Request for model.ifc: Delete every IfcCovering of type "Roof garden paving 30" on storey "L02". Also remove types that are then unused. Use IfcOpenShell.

First a look at what the model holds.

```python
import ifcopenshell
import ifcopenshell.util.element

model = ifcopenshell.open("model.ifc")
print(model.schema)
storey = next(s for s in model.by_type("IfcBuildingStorey") if s.Name == "L02")
coverings = [e for e in ifcopenshell.util.element.get_decomposition(storey) if e.is_a("IfcCovering")]
seen = {}
for e in coverings:
    element_type = ifcopenshell.util.element.get_type(e)
    name = element_type.Name if element_type not in (None, e) else None
    seen[name] = seen.get(name, 0) + 1
for name, count in sorted(seen.items(), key=str):
    print(count, "x", name)
```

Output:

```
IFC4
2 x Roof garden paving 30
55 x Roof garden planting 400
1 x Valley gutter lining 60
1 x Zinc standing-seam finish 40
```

```python
import ifcopenshell
import ifcopenshell.api.root
import ifcopenshell.util.element

model = ifcopenshell.open("model.ifc")

storey = next(s for s in model.by_type("IfcBuildingStorey") if s.Name == "L02")
coverings = [e for e in ifcopenshell.util.element.get_decomposition(storey) if e.is_a("IfcCovering")]
targets = [e for e in coverings if (t := ifcopenshell.util.element.get_type(e)) not in (None, e) and t.Name == "Roof garden paving 30"]
types = {ifcopenshell.util.element.get_type(e) for e in targets} - {None, *targets}

for e in targets:
    ifcopenshell.api.root.remove_product(model, product=e)
print(len(targets), "removed")

unused = [t for t in types if not ifcopenshell.util.element.get_types(t)]
for t in unused:
    ifcopenshell.api.root.remove_product(model, product=t)
print(len(unused), "unused types removed")

model.write("model_edited.ifc")
```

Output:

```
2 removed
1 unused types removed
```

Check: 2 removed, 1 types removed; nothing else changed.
